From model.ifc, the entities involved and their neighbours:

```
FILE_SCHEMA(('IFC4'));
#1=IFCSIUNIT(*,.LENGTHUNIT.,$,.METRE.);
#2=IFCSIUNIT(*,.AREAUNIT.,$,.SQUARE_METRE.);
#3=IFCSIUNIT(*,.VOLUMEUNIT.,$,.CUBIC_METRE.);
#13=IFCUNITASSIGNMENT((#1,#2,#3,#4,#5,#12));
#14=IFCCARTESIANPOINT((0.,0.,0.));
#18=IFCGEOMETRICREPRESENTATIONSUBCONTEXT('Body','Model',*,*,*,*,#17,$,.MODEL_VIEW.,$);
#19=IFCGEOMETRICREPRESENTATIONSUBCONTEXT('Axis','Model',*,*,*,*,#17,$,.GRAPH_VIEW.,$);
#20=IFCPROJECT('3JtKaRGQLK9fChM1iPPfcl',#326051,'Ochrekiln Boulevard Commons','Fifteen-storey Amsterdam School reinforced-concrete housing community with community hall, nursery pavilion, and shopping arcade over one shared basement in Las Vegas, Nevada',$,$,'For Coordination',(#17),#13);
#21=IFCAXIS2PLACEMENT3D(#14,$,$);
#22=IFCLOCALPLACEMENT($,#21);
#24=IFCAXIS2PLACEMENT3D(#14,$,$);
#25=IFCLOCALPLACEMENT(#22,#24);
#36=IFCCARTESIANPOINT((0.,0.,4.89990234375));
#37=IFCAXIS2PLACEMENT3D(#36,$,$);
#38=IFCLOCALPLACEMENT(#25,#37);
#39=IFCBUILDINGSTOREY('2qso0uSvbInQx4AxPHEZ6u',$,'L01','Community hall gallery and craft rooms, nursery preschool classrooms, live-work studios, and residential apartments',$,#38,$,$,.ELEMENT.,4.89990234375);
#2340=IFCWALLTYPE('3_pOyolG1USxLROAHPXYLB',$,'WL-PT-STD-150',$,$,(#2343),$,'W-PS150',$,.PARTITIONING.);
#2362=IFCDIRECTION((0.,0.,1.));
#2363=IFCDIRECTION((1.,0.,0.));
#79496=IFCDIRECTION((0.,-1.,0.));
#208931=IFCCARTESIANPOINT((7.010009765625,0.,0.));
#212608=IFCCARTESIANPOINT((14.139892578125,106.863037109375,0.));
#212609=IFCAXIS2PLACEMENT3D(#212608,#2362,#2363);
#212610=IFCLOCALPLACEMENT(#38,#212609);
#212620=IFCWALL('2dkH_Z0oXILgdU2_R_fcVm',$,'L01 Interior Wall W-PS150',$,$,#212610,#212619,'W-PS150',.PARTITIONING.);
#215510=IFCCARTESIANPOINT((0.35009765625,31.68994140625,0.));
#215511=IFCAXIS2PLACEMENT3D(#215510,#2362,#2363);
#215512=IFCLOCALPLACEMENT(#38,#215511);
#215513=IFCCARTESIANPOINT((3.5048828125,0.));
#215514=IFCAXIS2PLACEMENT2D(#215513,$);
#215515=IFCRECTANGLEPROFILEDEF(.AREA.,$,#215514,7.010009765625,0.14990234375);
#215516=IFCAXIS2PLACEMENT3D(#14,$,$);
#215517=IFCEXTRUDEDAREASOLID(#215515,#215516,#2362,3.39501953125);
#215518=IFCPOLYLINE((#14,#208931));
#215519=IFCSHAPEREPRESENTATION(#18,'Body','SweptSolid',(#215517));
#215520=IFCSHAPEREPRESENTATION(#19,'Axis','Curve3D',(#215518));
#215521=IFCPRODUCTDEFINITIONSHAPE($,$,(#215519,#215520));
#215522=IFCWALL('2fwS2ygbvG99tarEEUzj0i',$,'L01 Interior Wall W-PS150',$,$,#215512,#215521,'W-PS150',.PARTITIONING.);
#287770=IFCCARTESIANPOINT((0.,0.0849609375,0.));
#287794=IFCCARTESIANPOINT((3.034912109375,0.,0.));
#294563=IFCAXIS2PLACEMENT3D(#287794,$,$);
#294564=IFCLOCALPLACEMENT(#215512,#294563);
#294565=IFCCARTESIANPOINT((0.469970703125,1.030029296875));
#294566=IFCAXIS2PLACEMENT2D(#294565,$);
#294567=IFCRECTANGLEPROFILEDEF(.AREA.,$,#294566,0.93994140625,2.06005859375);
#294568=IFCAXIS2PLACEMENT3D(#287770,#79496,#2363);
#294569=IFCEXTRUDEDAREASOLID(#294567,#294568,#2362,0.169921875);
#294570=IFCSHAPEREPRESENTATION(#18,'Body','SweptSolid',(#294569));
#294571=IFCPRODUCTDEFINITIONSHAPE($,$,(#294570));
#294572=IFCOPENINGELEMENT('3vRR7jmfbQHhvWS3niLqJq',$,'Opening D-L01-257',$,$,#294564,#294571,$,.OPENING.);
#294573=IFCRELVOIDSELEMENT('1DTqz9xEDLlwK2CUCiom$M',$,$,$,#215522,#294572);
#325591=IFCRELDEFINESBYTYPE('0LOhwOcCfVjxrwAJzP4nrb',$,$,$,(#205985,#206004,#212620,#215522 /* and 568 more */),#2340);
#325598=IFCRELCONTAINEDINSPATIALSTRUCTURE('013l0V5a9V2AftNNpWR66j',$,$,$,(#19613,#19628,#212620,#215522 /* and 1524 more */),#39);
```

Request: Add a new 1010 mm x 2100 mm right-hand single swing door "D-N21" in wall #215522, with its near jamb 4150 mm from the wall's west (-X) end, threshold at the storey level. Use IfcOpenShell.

```python
import numpy as np
import ifcopenshell
import ifcopenshell.api.feature
import ifcopenshell.api.geometry
import ifcopenshell.api.root
import ifcopenshell.api.spatial
import ifcopenshell.geom
import ifcopenshell.util.element
import ifcopenshell.util.placement
import ifcopenshell.util.representation
import ifcopenshell.util.shape
import ifcopenshell.util.unit

model = ifcopenshell.open("model.ifc")
unit_scale = ifcopenshell.util.unit.calculate_unit_scale(model)
settings = ifcopenshell.geom.settings()


def volume(element):
    """Net volume in cubic metres, openings subtracted."""
    shape = ifcopenshell.geom.create_shape(settings, element)
    return ifcopenshell.util.shape.get_volume(shape.geometry)


wall = model.by_id(215522)
storey = ifcopenshell.util.element.get_container(wall, ifc_class="IfcBuildingStorey")
context = ifcopenshell.util.representation.get_context(model, "Model", "Body", "MODEL_VIEW")
before = volume(wall)

width, height, from_end, sill = 1.01, 2.1, 4.15, 0.0  # metres

# The wall runs along its own X axis, and the end named is its -X end.
wall_shape = ifcopenshell.geom.create_shape(settings, wall)
x, y, z = ifcopenshell.util.shape.get_vertices(wall_shape.geometry).T
start = x.min() + from_end
face, thickness = float(y.min()), float(y.max() - y.min())
wall_matrix = ifcopenshell.util.placement.get_local_placement(wall.ObjectPlacement)
level = ifcopenshell.util.placement.get_local_placement(storey.ObjectPlacement)[2, 3]


def in_wall(x, y):
    """Placement at x, y metres in the wall's axes, at sill height."""
    matrix = wall_matrix.copy()
    matrix[:, 3] = wall_matrix @ np.array([x / unit_scale, y / unit_scale, 0.0, 1.0])
    matrix[2, 3] = level + sill / unit_scale
    return matrix


# Opening: a box that overshoots both wall faces by 50 mm.
opening = ifcopenshell.api.root.create_entity(model, ifc_class="IfcOpeningElement", predefined_type="OPENING")
box = ifcopenshell.api.geometry.add_wall_representation(
    model, context=context, length=width, height=height, thickness=thickness + 0.1
)
ifcopenshell.api.geometry.assign_representation(model, product=opening, representation=box)
ifcopenshell.api.geometry.edit_object_placement(model, product=opening, matrix=in_wall(start, face - 0.05), is_si=False)
ifcopenshell.api.feature.add_feature(model, feature=opening, element=wall)

door = ifcopenshell.api.root.create_entity(model, ifc_class="IfcDoor", name="D-N21", predefined_type="DOOR")
door.OverallWidth, door.OverallHeight = width / unit_scale, height / unit_scale
door.OperationType = "SINGLE_SWING_RIGHT"
body = ifcopenshell.api.geometry.add_door_representation(
    model,
    context=context,
    overall_width=door.OverallWidth,
    overall_height=door.OverallHeight,
    operation_type="SINGLE_SWING_RIGHT",
    lining_properties={"LiningDepth": thickness / unit_scale, "ThresholdDepth": thickness / unit_scale},
)
ifcopenshell.api.geometry.assign_representation(model, product=door, representation=body)
ifcopenshell.api.spatial.assign_container(model, products=[door], relating_structure=storey)
ifcopenshell.api.feature.add_filling(model, opening=opening, element=door)

# The lining spans the wall, so the door starts at the wall face.
ifcopenshell.api.geometry.edit_object_placement(model, product=door, matrix=in_wall(start, face), is_si=False)

after = volume(wall)

print(f"wall volume {before:.3f} -> {after:.3f} m3")

model.write("model-out.ifc")
```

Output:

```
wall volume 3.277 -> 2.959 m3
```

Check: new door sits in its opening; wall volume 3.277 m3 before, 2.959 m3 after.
